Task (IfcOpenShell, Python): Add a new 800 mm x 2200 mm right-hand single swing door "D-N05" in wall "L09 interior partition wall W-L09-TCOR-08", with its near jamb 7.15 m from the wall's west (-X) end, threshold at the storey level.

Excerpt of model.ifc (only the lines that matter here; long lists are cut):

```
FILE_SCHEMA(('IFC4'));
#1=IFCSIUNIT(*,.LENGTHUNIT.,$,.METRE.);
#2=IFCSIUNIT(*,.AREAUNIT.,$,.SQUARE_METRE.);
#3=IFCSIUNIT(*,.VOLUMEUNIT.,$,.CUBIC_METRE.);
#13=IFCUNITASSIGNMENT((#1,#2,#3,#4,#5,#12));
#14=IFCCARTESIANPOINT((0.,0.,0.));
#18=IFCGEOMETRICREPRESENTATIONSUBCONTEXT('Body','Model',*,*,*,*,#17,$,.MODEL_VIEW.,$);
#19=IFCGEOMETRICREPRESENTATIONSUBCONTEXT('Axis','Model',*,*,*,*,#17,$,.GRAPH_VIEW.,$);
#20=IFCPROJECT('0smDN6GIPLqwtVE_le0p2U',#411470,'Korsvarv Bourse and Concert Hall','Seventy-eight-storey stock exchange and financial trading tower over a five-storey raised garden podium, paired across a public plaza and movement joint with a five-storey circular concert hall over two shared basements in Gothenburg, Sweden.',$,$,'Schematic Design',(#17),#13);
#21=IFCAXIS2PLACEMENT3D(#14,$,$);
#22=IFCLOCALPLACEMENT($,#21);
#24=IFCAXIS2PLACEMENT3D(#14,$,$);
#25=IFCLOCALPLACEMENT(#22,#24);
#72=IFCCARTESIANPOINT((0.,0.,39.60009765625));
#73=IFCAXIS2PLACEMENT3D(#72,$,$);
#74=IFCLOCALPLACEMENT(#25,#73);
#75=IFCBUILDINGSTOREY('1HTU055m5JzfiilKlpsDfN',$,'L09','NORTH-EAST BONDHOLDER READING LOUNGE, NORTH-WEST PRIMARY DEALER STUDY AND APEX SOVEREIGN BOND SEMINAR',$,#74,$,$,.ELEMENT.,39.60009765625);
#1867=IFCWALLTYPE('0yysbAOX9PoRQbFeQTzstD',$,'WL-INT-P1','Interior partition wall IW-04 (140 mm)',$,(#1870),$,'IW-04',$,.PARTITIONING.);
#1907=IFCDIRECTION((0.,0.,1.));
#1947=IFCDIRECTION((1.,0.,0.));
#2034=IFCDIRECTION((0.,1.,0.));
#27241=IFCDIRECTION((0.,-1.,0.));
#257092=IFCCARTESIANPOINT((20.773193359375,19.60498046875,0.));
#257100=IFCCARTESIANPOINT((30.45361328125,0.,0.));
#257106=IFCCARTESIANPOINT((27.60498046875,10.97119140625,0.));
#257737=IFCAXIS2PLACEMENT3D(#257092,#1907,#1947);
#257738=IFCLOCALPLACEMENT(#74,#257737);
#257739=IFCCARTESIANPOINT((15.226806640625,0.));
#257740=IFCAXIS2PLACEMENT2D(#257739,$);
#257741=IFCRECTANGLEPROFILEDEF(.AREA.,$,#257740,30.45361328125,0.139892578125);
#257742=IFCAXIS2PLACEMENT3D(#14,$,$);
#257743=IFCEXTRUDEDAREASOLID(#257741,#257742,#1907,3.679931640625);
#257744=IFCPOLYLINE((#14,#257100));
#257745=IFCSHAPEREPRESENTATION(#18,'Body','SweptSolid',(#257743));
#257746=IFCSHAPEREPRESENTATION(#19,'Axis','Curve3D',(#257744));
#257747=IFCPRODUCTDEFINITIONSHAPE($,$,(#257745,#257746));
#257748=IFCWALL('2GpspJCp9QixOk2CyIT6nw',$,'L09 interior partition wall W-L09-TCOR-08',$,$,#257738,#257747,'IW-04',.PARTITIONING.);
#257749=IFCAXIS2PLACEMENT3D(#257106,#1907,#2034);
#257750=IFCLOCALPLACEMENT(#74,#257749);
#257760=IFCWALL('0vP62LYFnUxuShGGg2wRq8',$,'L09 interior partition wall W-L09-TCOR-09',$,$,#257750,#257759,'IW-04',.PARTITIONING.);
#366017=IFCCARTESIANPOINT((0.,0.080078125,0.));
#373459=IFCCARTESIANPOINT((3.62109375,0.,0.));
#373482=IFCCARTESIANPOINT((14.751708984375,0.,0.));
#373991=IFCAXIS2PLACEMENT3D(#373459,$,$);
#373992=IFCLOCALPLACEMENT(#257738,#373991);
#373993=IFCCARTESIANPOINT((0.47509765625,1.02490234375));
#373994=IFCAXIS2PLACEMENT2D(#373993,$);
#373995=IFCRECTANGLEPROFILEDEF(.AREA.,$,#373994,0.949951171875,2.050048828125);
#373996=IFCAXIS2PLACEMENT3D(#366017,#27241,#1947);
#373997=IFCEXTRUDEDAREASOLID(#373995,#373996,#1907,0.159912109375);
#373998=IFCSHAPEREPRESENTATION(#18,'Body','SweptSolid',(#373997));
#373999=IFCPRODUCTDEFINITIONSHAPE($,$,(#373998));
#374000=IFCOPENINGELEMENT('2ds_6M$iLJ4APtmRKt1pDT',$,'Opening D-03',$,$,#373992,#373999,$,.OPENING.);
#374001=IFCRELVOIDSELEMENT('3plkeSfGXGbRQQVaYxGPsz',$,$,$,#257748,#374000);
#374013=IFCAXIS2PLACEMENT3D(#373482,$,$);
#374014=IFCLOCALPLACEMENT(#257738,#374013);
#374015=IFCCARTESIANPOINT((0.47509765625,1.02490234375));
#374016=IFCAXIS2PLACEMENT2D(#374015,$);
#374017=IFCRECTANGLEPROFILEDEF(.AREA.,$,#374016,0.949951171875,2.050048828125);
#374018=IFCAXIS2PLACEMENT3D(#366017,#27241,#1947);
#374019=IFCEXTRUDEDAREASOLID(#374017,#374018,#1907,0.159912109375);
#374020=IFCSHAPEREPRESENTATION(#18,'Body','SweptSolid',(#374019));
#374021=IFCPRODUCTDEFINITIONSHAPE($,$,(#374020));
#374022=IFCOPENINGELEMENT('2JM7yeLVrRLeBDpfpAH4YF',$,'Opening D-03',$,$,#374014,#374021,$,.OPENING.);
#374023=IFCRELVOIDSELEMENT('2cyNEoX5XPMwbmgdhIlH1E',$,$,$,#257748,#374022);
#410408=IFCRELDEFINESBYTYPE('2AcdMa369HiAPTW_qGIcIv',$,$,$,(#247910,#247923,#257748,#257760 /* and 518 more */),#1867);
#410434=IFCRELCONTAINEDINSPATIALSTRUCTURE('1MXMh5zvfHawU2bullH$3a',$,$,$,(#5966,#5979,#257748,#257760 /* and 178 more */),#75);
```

```python
import numpy as np
import ifcopenshell
import ifcopenshell.api.feature
import ifcopenshell.api.geometry
import ifcopenshell.api.root
import ifcopenshell.api.spatial
import ifcopenshell.geom
import ifcopenshell.util.element
import ifcopenshell.util.placement
import ifcopenshell.util.representation
import ifcopenshell.util.shape
import ifcopenshell.util.unit

model = ifcopenshell.open("model.ifc")
unit_scale = ifcopenshell.util.unit.calculate_unit_scale(model)
settings = ifcopenshell.geom.settings()


def volume(element):
    """Net volume in cubic metres, openings subtracted."""
    shape = ifcopenshell.geom.create_shape(settings, element)
    return ifcopenshell.util.shape.get_volume(shape.geometry)


wall = model.by_guid("2GpspJCp9QixOk2CyIT6nw")
storey = ifcopenshell.util.element.get_container(wall, ifc_class="IfcBuildingStorey")
context = ifcopenshell.util.representation.get_context(model, "Model", "Body", "MODEL_VIEW")
before = volume(wall)

width, height, from_end, sill = 0.8, 2.2, 7.15, 0.0  # metres

# The wall runs along its own X axis, and the end named is its -X end.
wall_shape = ifcopenshell.geom.create_shape(settings, wall)
x, y, z = ifcopenshell.util.shape.get_vertices(wall_shape.geometry).T
start = x.min() + from_end
face, thickness = float(y.min()), float(y.max() - y.min())
wall_matrix = ifcopenshell.util.placement.get_local_placement(wall.ObjectPlacement)
level = ifcopenshell.util.placement.get_local_placement(storey.ObjectPlacement)[2, 3]


def in_wall(x, y):
    """Placement at x, y metres in the wall's axes, at sill height."""
    matrix = wall_matrix.copy()
    matrix[:, 3] = wall_matrix @ np.array([x / unit_scale, y / unit_scale, 0.0, 1.0])
    matrix[2, 3] = level + sill / unit_scale
    return matrix


# Opening: a box that overshoots both wall faces by 50 mm.
opening = ifcopenshell.api.root.create_entity(model, ifc_class="IfcOpeningElement", predefined_type="OPENING")
box = ifcopenshell.api.geometry.add_wall_representation(
    model, context=context, length=width, height=height, thickness=thickness + 0.1
)
ifcopenshell.api.geometry.assign_representation(model, product=opening, representation=box)
ifcopenshell.api.geometry.edit_object_placement(model, product=opening, matrix=in_wall(start, face - 0.05), is_si=False)
ifcopenshell.api.feature.add_feature(model, feature=opening, element=wall)

door = ifcopenshell.api.root.create_entity(model, ifc_class="IfcDoor", name="D-N05", predefined_type="DOOR")
door.OverallWidth, door.OverallHeight = width / unit_scale, height / unit_scale
door.OperationType = "SINGLE_SWING_RIGHT"
body = ifcopenshell.api.geometry.add_door_representation(
    model,
    context=context,
    overall_width=door.OverallWidth,
    overall_height=door.OverallHeight,
    operation_type="SINGLE_SWING_RIGHT",
    lining_properties={"LiningDepth": thickness / unit_scale, "ThresholdDepth": thickness / unit_scale},
)
ifcopenshell.api.geometry.assign_representation(model, product=door, representation=body)
ifcopenshell.api.spatial.assign_container(model, products=[door], relating_structure=storey)
ifcopenshell.api.feature.add_filling(model, opening=opening, element=door)

# The lining spans the wall, so the door starts at the wall face.
ifcopenshell.api.geometry.edit_object_placement(model, product=door, matrix=in_wall(start, face), is_si=False)

after = volume(wall)

print(f"wall volume {before:.3f} -> {after:.3f} m3")

model.write("model_updated.ifc")
```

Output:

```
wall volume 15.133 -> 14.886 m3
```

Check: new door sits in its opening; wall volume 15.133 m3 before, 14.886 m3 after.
